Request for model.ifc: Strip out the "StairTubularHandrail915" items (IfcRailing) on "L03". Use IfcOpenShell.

First a look at what the model holds.

```python
import ifcopenshell
import ifcopenshell.util.element

model = ifcopenshell.open("model.ifc")
print(model.schema)
storey = next(s for s in model.by_type("IfcBuildingStorey") if s.Name == "L03")
railings = [e for e in ifcopenshell.util.element.get_decomposition(storey) if e.is_a("IfcRailing")]
seen = {}
for e in railings:
    element_type = ifcopenshell.util.element.get_type(e)
    name = element_type.Name if element_type not in (None, e) else None
    seen[name] = seen.get(name, 0) + 1
for name, count in sorted(seen.items(), key=str):
    print(count, "x", name)
```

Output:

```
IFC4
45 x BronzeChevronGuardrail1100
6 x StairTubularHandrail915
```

```python
import ifcopenshell
import ifcopenshell.api.root
import ifcopenshell.util.element

model = ifcopenshell.open("model.ifc")

storey = next(s for s in model.by_type("IfcBuildingStorey") if s.Name == "L03")
railings = [e for e in ifcopenshell.util.element.get_decomposition(storey) if e.is_a("IfcRailing")]
targets = [e for e in railings if (t := ifcopenshell.util.element.get_type(e)) not in (None, e) and t.Name == "StairTubularHandrail915"]

for e in targets:
    ifcopenshell.api.root.remove_product(model, product=e)
print(len(targets), "removed")

model.write("model-out.ifc")
```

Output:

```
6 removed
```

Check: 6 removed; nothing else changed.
